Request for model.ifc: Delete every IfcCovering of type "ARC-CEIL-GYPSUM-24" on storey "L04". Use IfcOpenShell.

First a look at what the model holds.

```python
import ifcopenshell
import ifcopenshell.util.element

model = ifcopenshell.open("model.ifc")
print(model.schema)
storey = next(s for s in model.by_type("IfcBuildingStorey") if s.Name == "L04")
coverings = [e for e in ifcopenshell.util.element.get_decomposition(storey) if e.is_a("IfcCovering")]
seen = {}
for e in coverings:
    element_type = ifcopenshell.util.element.get_type(e)
    name = element_type.Name if element_type not in (None, e) else None
    seen[name] = seen.get(name, 0) + 1
for name, count in sorted(seen.items(), key=str):
    print(count, "x", name)
```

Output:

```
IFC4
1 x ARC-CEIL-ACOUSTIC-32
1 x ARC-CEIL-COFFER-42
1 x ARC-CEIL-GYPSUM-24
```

```python
import ifcopenshell
import ifcopenshell.api.root
import ifcopenshell.util.element

model = ifcopenshell.open("model.ifc")

storey = next(s for s in model.by_type("IfcBuildingStorey") if s.Name == "L04")
coverings = [e for e in ifcopenshell.util.element.get_decomposition(storey) if e.is_a("IfcCovering")]
targets = [e for e in coverings if (t := ifcopenshell.util.element.get_type(e)) not in (None, e) and t.Name == "ARC-CEIL-GYPSUM-24"]

for e in targets:
    ifcopenshell.api.root.remove_product(model, product=e)
print(len(targets), "removed")

model.write("model_v2.ifc")
```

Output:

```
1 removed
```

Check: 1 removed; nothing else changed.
